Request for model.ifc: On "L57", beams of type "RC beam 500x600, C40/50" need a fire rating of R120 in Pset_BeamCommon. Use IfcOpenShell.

First a look at what the model holds.

```python
import ifcopenshell
import ifcopenshell.util.element

model = ifcopenshell.open("model.ifc")
print(model.schema)
storey = next(s for s in model.by_type("IfcBuildingStorey") if s.Name == "L57")
beams = [e for e in ifcopenshell.util.element.get_decomposition(storey) if e.is_a("IfcBeam")]
seen = {}
for e in beams:
    element_type = ifcopenshell.util.element.get_type(e)
    key = (element_type.Name if element_type != e and element_type else None, ifcopenshell.util.element.get_pset(e, "Pset_BeamCommon", "FireRating"))
    seen[key] = seen.get(key, 0) + 1
for (name, value), count in sorted(seen.items(), key=str):
    print(count, "x", name, "|", value)
```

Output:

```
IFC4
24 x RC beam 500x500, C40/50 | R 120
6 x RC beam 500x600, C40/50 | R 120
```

```python
import ifcopenshell
import ifcopenshell.api.pset
import ifcopenshell.util.element

model = ifcopenshell.open("model.ifc")

storey = next(s for s in model.by_type("IfcBuildingStorey") if s.Name == "L57")
beams = [e for e in ifcopenshell.util.element.get_decomposition(storey) if e.is_a("IfcBeam")]

count = 0
for e in beams:
    element_type = ifcopenshell.util.element.get_type(e)
    if element_type in (None, e) or element_type.Name != "RC beam 500x600, C40/50":
        continue
    found = ifcopenshell.util.element.get_pset(e, "Pset_BeamCommon", should_inherit=False)
    if found:
        pset = model.by_id(found["id"])
        if len(ifcopenshell.util.element.get_elements_by_pset(pset)) > 1:
            pset = ifcopenshell.api.pset.unshare_pset(model, products=[e], pset=pset)[0]
    else:
        pset = ifcopenshell.api.pset.add_pset(model, product=e, name="Pset_BeamCommon")
    ifcopenshell.api.pset.edit_pset(model, pset=pset, properties={"FireRating": "R120"})
    count += 1

print(count, "beams updated")

model.write("model-out.ifc")
```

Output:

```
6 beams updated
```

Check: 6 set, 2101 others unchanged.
